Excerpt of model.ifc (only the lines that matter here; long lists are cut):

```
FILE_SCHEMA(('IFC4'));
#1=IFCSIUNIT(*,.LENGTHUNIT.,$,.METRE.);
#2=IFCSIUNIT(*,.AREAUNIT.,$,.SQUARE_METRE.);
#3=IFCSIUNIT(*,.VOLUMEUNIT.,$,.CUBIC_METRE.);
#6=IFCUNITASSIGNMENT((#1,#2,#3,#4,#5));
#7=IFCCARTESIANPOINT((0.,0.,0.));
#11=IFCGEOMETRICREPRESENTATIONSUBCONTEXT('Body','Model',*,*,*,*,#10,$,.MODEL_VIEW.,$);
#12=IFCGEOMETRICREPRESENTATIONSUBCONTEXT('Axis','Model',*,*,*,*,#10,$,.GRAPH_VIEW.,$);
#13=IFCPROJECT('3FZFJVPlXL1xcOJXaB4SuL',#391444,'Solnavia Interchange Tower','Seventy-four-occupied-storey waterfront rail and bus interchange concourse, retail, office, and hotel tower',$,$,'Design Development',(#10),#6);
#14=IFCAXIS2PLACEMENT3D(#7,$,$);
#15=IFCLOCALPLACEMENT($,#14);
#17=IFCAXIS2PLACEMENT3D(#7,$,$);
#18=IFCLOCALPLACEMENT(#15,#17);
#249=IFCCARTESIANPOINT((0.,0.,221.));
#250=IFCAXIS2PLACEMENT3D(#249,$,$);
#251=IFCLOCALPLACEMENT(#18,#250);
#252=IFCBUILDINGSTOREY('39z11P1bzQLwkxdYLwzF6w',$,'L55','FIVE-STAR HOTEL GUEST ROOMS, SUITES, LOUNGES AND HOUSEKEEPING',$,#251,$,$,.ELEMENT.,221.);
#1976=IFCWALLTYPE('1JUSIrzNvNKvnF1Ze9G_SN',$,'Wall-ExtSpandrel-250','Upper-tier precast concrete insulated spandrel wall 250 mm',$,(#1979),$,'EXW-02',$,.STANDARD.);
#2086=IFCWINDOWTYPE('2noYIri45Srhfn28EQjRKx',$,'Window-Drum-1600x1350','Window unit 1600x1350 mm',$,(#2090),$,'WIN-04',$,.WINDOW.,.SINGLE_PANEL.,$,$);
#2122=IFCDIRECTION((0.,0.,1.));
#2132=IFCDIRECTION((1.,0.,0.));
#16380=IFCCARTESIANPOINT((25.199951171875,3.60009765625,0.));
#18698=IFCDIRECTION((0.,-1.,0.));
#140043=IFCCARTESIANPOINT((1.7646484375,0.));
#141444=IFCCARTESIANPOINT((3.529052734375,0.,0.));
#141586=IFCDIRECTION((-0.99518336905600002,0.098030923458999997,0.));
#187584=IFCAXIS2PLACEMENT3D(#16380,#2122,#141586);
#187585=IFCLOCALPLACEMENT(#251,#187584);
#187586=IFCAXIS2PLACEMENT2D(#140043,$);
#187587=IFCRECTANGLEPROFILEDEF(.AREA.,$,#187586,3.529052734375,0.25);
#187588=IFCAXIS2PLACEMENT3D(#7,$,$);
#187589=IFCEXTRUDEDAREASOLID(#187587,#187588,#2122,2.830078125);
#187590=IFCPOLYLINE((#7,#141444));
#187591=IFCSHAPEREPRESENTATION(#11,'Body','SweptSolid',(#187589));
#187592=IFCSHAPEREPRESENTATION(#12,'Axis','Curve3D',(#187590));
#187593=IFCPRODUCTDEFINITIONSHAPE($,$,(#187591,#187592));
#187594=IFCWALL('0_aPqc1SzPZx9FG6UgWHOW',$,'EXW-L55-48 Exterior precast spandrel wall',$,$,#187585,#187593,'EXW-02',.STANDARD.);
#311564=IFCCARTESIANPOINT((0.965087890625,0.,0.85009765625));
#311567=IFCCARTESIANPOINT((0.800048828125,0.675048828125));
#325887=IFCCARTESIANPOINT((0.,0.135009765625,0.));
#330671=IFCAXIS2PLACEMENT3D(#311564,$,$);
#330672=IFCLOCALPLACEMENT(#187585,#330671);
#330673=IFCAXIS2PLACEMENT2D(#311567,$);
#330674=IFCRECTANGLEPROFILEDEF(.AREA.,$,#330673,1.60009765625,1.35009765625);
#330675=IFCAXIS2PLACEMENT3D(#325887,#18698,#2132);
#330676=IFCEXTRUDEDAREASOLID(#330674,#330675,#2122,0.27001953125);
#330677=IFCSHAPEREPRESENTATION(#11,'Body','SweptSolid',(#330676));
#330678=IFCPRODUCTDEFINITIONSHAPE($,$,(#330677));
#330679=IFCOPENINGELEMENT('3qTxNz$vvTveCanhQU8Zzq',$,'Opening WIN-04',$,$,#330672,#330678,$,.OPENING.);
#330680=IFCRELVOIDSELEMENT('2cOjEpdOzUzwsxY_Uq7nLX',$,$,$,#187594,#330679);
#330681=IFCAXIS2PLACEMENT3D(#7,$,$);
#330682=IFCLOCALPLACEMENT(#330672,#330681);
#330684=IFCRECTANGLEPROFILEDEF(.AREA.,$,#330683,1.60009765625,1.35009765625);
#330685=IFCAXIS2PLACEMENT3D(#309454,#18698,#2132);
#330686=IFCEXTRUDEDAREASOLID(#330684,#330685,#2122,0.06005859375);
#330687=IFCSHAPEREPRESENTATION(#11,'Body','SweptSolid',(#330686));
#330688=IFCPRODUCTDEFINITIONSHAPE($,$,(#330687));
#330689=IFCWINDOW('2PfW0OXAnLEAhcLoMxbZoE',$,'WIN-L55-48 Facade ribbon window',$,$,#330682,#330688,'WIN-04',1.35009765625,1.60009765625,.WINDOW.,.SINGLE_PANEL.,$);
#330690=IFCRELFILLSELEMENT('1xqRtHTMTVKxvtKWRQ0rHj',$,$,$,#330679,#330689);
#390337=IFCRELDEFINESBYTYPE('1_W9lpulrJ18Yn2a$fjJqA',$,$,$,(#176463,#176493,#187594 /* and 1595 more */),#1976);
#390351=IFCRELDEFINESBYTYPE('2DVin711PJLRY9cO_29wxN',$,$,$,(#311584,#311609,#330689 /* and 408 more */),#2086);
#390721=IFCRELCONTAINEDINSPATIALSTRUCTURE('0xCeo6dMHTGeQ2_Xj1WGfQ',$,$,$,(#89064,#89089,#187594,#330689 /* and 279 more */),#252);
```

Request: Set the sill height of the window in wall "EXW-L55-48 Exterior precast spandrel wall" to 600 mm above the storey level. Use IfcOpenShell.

```python
import numpy as np
import ifcopenshell
import ifcopenshell.api.geometry
import ifcopenshell.geom
import ifcopenshell.util.element
import ifcopenshell.util.placement
import ifcopenshell.util.shape
import ifcopenshell.util.unit

model = ifcopenshell.open("model.ifc")
unit_scale = ifcopenshell.util.unit.calculate_unit_scale(model)

window = model.by_guid("2PfW0OXAnLEAhcLoMxbZoE")
opening = window.FillsVoids[0].RelatingOpeningElement
storey = ifcopenshell.util.element.get_container(window, ifc_class="IfcBuildingStorey")
level = ifcopenshell.util.placement.get_local_placement(storey.ObjectPlacement)[2, 3]

# The opening's origin need not be at the sill, so measure its lowest point.
shape = ifcopenshell.geom.create_shape(ifcopenshell.geom.settings(), opening)
bottom = ifcopenshell.util.shape.get_shape_bottom_elevation(shape, shape.geometry) / unit_scale
dz = level + 0.6 / unit_scale - bottom

shift = np.array([0.0, 0.0, dz])
# The window is placed relative to its opening, so it follows when the opening moves.
matrix = ifcopenshell.util.placement.get_local_placement(opening.ObjectPlacement)
matrix[:3, 3] += shift
ifcopenshell.api.geometry.edit_object_placement(
    model, product=opening, matrix=matrix, is_si=False, should_transform_children=True
)

print(f"moved by {dz * unit_scale:+.3f} m")

model.write("model_edited.ifc")
```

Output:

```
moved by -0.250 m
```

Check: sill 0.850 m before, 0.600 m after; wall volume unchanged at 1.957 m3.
